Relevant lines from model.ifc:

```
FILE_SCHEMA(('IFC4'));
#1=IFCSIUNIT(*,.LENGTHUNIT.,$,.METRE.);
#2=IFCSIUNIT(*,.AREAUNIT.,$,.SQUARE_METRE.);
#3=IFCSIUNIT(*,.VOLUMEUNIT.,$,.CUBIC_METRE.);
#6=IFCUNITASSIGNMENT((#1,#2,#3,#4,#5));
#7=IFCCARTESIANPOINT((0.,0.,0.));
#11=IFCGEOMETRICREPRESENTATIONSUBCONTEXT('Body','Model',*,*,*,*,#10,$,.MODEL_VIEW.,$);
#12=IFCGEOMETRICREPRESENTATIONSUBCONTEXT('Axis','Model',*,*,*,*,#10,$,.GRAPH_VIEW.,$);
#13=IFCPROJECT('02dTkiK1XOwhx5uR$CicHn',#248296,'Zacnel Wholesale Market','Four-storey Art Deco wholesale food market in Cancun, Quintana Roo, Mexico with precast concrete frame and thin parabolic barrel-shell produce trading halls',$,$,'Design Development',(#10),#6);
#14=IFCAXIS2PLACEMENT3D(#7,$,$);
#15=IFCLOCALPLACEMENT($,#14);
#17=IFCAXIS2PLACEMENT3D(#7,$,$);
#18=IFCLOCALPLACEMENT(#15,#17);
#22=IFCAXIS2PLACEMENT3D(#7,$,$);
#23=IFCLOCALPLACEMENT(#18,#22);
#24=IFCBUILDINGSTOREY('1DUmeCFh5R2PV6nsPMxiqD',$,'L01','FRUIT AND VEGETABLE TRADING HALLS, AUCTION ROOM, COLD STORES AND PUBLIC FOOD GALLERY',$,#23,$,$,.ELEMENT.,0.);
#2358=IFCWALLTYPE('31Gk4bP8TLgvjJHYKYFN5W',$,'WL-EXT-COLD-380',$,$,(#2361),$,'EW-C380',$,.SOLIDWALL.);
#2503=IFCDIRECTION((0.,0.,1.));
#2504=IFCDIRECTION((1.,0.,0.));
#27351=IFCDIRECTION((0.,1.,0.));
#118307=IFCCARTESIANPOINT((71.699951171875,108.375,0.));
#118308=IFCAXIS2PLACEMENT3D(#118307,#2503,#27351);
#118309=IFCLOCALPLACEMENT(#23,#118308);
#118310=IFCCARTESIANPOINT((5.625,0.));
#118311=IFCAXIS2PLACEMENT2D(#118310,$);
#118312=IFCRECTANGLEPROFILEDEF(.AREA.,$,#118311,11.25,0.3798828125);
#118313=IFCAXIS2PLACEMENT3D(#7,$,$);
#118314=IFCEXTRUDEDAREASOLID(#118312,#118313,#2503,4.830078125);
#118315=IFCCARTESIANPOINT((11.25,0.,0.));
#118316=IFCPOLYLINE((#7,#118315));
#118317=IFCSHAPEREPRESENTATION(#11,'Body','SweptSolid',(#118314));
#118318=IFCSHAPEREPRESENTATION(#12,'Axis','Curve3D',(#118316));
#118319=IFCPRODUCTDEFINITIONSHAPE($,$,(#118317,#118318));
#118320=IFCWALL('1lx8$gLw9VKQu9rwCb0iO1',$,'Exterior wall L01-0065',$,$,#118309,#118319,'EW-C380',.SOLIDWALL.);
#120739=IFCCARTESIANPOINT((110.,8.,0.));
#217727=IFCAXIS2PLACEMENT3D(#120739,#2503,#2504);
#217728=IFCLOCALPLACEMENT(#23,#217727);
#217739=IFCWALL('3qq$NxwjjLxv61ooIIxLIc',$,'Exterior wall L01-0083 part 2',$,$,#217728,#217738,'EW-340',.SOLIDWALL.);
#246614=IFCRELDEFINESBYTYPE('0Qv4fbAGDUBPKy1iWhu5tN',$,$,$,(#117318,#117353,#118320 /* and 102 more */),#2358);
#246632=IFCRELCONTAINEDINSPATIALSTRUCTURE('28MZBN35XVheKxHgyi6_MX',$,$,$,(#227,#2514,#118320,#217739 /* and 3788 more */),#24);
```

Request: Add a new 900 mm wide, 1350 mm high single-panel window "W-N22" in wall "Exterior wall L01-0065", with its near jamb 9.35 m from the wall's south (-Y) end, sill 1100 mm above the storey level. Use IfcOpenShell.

```python
import numpy as np
import ifcopenshell
import ifcopenshell.api.feature
import ifcopenshell.api.geometry
import ifcopenshell.api.root
import ifcopenshell.api.spatial
import ifcopenshell.geom
import ifcopenshell.util.element
import ifcopenshell.util.placement
import ifcopenshell.util.representation
import ifcopenshell.util.shape
import ifcopenshell.util.unit

model = ifcopenshell.open("model.ifc")
unit_scale = ifcopenshell.util.unit.calculate_unit_scale(model)
settings = ifcopenshell.geom.settings()


def volume(element):
    """Net volume in cubic metres, openings subtracted."""
    shape = ifcopenshell.geom.create_shape(settings, element)
    return ifcopenshell.util.shape.get_volume(shape.geometry)


wall = model.by_id(118320)
storey = ifcopenshell.util.element.get_container(wall, ifc_class="IfcBuildingStorey")
context = ifcopenshell.util.representation.get_context(model, "Model", "Body", "MODEL_VIEW")
before = volume(wall)

width, height, from_end, sill = 0.9, 1.35, 9.35, 1.1  # metres

# The wall runs along its own X axis, and the end named is its -X end.
wall_shape = ifcopenshell.geom.create_shape(settings, wall)
x, y, z = ifcopenshell.util.shape.get_vertices(wall_shape.geometry).T
start = x.min() + from_end
face, thickness = float(y.min()), float(y.max() - y.min())
wall_matrix = ifcopenshell.util.placement.get_local_placement(wall.ObjectPlacement)
level = ifcopenshell.util.placement.get_local_placement(storey.ObjectPlacement)[2, 3]


def in_wall(x, y):
    """Placement at x, y metres in the wall's axes, at sill height."""
    matrix = wall_matrix.copy()
    matrix[:, 3] = wall_matrix @ np.array([x / unit_scale, y / unit_scale, 0.0, 1.0])
    matrix[2, 3] = level + sill / unit_scale
    return matrix


# Opening: a box that overshoots both wall faces by 50 mm.
opening = ifcopenshell.api.root.create_entity(model, ifc_class="IfcOpeningElement", predefined_type="OPENING")
box = ifcopenshell.api.geometry.add_wall_representation(
    model, context=context, length=width, height=height, thickness=thickness + 0.1
)
ifcopenshell.api.geometry.assign_representation(model, product=opening, representation=box)
ifcopenshell.api.geometry.edit_object_placement(model, product=opening, matrix=in_wall(start, face - 0.05), is_si=False)
ifcopenshell.api.feature.add_feature(model, feature=opening, element=wall)

window = ifcopenshell.api.root.create_entity(model, ifc_class="IfcWindow", name="W-N22", predefined_type="WINDOW")
window.OverallWidth, window.OverallHeight = width / unit_scale, height / unit_scale
window.PartitioningType = "SINGLE_PANEL"
body = ifcopenshell.api.geometry.add_window_representation(
    model,
    context=context,
    overall_width=window.OverallWidth,
    overall_height=window.OverallHeight,
    partition_type="SINGLE_PANEL",
)
ifcopenshell.api.geometry.assign_representation(model, product=window, representation=body)
ifcopenshell.api.spatial.assign_container(model, products=[window], relating_structure=storey)
ifcopenshell.api.feature.add_filling(model, opening=opening, element=window)

# Centre the window in the wall's thickness.
ifcopenshell.api.geometry.edit_object_placement(model, product=window, matrix=in_wall(start, face), is_si=False)
window_shape = ifcopenshell.geom.create_shape(settings, window)
depth = ifcopenshell.util.shape.get_vertices(window_shape.geometry)[:, 1]
offset = face + thickness / 2 - (depth.min() + depth.max()) / 2
ifcopenshell.api.geometry.edit_object_placement(model, product=window, matrix=in_wall(start, offset), is_si=False)

after = volume(wall)

print(f"wall volume {before:.3f} -> {after:.3f} m3")

model.write("model_updated.ifc")
```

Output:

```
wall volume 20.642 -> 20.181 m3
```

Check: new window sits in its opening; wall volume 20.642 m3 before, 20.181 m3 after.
